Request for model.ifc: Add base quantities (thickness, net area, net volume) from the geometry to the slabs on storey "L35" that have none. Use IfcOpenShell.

First a look at what the model holds.

```python
import ifcopenshell
import ifcopenshell.util.element
import ifcopenshell.util.unit

model = ifcopenshell.open("model.ifc")
print(model.schema)
for unit_type in ("LENGTHUNIT", "AREAUNIT", "VOLUMEUNIT"):
    print(unit_type, ifcopenshell.util.unit.calculate_unit_scale(model, unit_type))
storey = next(s for s in model.by_type("IfcBuildingStorey") if s.Name == "L35")
slabs = [e for e in ifcopenshell.util.element.get_decomposition(storey) if e.is_a("IfcSlab")]
for e in sorted(slabs, key=lambda e: e.id()):
    print(e.id(), e.is_a(), e.Name, list(ifcopenshell.util.element.get_psets(e, qtos_only=True)), sep=" | ")
```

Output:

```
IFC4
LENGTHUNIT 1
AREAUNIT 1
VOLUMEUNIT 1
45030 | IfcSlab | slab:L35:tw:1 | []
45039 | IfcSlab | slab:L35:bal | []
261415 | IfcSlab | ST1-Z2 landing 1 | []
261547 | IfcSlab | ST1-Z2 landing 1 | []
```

```python
import ifcopenshell
import ifcopenshell.api.pset
import ifcopenshell.geom
import ifcopenshell.util.element
import ifcopenshell.util.shape
import ifcopenshell.util.unit

model = ifcopenshell.open("model.ifc")
unit_scale = ifcopenshell.util.unit.calculate_unit_scale(model)
area_scale = ifcopenshell.util.unit.calculate_unit_scale(model, "AREAUNIT")
volume_scale = ifcopenshell.util.unit.calculate_unit_scale(model, "VOLUMEUNIT")
settings = ifcopenshell.geom.settings()

storey = next(s for s in model.by_type("IfcBuildingStorey") if s.Name == "L35")
slabs = [e for e in ifcopenshell.util.element.get_decomposition(storey) if e.is_a("IfcSlab")]

for e in sorted(slabs, key=lambda e: e.id()):
    if ifcopenshell.util.element.get_psets(e, qtos_only=True, should_inherit=False):
        continue
    # Geometry comes back in metres, in the element's own axes.
    shape = ifcopenshell.geom.create_shape(settings, e)
    values = {
        "Width": ifcopenshell.util.shape.get_z(shape.geometry) / unit_scale,
        "NetArea": ifcopenshell.util.shape.get_footprint_area(shape.geometry) / area_scale,
        "NetVolume": ifcopenshell.util.shape.get_volume(shape.geometry) / volume_scale,
    }
    qto = ifcopenshell.api.pset.add_qto(model, product=e, name="Qto_SlabBaseQuantities")
    ifcopenshell.api.pset.edit_qto(model, qto=qto, properties=values)
    print(e.id(), {k: round(v, 3) for k, v in values.items()})

model.write("model-out.ifc")
```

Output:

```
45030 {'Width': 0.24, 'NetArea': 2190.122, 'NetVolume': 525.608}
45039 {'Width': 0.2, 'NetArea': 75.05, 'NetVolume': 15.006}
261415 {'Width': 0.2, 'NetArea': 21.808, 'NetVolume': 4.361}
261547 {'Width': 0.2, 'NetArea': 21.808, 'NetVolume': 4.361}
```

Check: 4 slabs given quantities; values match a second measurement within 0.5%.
